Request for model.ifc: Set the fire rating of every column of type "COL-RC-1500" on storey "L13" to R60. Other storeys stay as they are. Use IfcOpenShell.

First a look at what the model holds.

```python
import ifcopenshell
import ifcopenshell.util.element

model = ifcopenshell.open("model.ifc")
print(model.schema)
storey = next(s for s in model.by_type("IfcBuildingStorey") if s.Name == "L13")
columns = [e for e in ifcopenshell.util.element.get_decomposition(storey) if e.is_a("IfcColumn")]
seen = {}
for e in columns:
    element_type = ifcopenshell.util.element.get_type(e)
    key = (element_type.Name if element_type != e and element_type else None, ifcopenshell.util.element.get_pset(e, "Pset_ColumnCommon", "FireRating"))
    seen[key] = seen.get(key, 0) + 1
for (name, value), count in sorted(seen.items(), key=str):
    print(count, "x", name, "|", value)
```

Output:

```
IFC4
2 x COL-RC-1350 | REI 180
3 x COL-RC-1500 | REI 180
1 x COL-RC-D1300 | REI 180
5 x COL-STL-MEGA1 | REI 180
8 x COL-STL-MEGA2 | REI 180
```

```python
import ifcopenshell
import ifcopenshell.api.pset
import ifcopenshell.util.element

model = ifcopenshell.open("model.ifc")

storey = next(s for s in model.by_type("IfcBuildingStorey") if s.Name == "L13")
columns = [e for e in ifcopenshell.util.element.get_decomposition(storey) if e.is_a("IfcColumn")]

count = 0
for e in columns:
    element_type = ifcopenshell.util.element.get_type(e)
    if element_type in (None, e) or element_type.Name != "COL-RC-1500":
        continue
    # add_pset returns the element's existing set when there is one.
    pset = ifcopenshell.api.pset.add_pset(model, product=e, name="Pset_ColumnCommon")
    ifcopenshell.api.pset.edit_pset(model, pset=pset, properties={"FireRating": "R60"})
    count += 1

print(count, "columns updated")

model.write("model_v2.ifc")
```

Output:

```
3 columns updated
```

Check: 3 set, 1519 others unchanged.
